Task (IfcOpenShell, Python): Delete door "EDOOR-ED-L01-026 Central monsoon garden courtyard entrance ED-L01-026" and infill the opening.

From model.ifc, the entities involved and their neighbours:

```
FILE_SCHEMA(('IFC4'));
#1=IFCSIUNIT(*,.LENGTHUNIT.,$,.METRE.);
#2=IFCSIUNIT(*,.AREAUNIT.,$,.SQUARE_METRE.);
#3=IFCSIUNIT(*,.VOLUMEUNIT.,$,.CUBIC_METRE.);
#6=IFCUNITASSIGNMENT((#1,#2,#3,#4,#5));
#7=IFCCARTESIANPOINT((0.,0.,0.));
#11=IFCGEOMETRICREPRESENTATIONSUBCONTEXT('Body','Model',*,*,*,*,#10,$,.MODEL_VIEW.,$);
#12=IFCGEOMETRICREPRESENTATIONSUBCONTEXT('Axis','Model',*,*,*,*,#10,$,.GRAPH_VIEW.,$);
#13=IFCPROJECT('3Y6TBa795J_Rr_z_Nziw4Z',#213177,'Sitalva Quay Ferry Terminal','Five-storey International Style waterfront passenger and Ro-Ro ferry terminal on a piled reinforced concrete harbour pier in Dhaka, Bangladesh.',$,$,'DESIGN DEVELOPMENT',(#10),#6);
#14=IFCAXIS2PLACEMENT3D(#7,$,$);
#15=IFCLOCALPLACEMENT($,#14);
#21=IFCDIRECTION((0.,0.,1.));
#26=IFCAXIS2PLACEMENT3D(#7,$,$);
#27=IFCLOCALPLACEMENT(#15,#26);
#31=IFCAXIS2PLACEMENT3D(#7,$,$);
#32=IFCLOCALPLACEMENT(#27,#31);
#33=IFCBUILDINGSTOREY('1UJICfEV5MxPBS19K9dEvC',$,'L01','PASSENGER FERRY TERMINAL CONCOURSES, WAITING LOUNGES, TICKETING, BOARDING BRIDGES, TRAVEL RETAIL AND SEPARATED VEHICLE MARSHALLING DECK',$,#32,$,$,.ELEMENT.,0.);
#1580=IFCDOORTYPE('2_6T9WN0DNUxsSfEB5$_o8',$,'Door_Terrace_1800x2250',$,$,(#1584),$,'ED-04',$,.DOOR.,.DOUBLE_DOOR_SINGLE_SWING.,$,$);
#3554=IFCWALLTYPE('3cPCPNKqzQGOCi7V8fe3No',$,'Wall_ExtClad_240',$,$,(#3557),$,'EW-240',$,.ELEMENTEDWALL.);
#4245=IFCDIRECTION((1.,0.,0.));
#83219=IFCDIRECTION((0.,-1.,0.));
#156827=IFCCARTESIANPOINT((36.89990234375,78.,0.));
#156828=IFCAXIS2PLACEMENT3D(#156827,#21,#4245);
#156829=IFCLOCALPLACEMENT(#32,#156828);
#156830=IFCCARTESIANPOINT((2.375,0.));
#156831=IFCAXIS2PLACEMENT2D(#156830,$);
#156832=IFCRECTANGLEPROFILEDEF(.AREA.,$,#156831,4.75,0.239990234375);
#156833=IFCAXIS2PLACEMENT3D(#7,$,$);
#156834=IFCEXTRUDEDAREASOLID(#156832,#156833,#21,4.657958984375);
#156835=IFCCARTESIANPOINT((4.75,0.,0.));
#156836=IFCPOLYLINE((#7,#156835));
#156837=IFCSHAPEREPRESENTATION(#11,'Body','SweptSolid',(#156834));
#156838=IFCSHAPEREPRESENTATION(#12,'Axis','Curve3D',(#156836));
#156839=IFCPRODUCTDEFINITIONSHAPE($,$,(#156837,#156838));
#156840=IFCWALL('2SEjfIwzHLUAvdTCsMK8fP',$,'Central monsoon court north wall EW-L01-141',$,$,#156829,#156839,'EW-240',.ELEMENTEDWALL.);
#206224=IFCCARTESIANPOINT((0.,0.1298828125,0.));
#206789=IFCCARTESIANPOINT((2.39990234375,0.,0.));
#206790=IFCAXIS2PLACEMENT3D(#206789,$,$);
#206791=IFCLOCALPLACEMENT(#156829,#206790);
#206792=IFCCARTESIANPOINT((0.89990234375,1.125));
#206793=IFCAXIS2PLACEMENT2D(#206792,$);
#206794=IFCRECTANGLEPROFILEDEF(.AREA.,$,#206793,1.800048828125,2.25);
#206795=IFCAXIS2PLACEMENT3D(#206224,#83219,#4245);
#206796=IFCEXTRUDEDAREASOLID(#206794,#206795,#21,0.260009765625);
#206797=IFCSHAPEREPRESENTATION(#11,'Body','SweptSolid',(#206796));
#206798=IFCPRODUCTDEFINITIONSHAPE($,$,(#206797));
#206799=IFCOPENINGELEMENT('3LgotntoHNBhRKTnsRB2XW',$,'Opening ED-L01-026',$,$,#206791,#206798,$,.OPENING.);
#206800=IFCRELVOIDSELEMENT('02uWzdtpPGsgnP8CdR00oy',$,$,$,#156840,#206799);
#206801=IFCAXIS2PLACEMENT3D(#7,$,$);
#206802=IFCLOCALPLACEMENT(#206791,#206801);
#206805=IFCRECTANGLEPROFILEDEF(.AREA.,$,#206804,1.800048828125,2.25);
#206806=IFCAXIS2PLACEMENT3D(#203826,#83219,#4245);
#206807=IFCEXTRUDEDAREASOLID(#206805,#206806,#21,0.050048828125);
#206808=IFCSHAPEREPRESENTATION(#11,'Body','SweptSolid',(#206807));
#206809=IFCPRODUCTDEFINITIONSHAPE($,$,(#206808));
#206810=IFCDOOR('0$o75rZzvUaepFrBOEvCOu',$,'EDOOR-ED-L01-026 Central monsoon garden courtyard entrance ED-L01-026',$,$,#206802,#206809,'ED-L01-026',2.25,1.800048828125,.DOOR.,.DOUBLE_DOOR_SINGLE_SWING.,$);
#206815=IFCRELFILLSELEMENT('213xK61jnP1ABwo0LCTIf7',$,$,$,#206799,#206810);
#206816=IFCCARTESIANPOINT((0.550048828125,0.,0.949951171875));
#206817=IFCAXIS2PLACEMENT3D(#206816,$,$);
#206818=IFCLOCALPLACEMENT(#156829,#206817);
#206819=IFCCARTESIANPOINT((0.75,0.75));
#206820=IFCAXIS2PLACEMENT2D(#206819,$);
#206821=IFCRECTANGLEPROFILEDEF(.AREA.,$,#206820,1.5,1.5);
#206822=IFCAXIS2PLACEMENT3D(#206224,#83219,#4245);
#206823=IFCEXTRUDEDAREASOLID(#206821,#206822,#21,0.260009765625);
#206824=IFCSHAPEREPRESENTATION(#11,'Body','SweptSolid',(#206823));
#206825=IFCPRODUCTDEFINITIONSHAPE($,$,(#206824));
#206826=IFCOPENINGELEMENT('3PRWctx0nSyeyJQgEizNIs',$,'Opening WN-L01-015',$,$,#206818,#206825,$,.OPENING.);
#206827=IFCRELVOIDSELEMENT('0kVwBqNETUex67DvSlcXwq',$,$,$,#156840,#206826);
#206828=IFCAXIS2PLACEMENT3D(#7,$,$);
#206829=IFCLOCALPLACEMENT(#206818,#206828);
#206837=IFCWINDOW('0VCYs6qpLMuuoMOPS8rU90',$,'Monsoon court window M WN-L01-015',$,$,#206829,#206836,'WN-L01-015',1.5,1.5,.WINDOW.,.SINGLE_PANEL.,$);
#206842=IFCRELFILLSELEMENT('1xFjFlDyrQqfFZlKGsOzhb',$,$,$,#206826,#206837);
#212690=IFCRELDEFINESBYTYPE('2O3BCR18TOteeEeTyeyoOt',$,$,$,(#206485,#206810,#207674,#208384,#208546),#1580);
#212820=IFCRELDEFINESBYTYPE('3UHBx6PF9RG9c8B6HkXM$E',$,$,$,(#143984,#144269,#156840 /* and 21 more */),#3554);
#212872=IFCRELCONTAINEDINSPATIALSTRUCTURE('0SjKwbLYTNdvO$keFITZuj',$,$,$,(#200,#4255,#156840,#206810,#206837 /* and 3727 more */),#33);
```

```python
import ifcopenshell
import ifcopenshell.api.feature
import ifcopenshell.api.root
import ifcopenshell.geom
import ifcopenshell.util.shape

model = ifcopenshell.open("model.ifc")
settings = ifcopenshell.geom.settings()


def volume(element):
    """Net volume in cubic metres, openings subtracted."""
    shape = ifcopenshell.geom.create_shape(settings, element)
    return ifcopenshell.util.shape.get_volume(shape.geometry)


door = model.by_id(206810)
opening = door.FillsVoids[0].RelatingOpeningElement
wall = opening.VoidsElements[0].RelatingBuildingElement
before = volume(wall)

ifcopenshell.api.root.remove_product(model, product=door)
ifcopenshell.api.feature.remove_feature(model, feature=opening)

after = volume(wall)

print(f"wall volume {before:.3f} -> {after:.3f} m3")

model.write("model_updated.ifc")
```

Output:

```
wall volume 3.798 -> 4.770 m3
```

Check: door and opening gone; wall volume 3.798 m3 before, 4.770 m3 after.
